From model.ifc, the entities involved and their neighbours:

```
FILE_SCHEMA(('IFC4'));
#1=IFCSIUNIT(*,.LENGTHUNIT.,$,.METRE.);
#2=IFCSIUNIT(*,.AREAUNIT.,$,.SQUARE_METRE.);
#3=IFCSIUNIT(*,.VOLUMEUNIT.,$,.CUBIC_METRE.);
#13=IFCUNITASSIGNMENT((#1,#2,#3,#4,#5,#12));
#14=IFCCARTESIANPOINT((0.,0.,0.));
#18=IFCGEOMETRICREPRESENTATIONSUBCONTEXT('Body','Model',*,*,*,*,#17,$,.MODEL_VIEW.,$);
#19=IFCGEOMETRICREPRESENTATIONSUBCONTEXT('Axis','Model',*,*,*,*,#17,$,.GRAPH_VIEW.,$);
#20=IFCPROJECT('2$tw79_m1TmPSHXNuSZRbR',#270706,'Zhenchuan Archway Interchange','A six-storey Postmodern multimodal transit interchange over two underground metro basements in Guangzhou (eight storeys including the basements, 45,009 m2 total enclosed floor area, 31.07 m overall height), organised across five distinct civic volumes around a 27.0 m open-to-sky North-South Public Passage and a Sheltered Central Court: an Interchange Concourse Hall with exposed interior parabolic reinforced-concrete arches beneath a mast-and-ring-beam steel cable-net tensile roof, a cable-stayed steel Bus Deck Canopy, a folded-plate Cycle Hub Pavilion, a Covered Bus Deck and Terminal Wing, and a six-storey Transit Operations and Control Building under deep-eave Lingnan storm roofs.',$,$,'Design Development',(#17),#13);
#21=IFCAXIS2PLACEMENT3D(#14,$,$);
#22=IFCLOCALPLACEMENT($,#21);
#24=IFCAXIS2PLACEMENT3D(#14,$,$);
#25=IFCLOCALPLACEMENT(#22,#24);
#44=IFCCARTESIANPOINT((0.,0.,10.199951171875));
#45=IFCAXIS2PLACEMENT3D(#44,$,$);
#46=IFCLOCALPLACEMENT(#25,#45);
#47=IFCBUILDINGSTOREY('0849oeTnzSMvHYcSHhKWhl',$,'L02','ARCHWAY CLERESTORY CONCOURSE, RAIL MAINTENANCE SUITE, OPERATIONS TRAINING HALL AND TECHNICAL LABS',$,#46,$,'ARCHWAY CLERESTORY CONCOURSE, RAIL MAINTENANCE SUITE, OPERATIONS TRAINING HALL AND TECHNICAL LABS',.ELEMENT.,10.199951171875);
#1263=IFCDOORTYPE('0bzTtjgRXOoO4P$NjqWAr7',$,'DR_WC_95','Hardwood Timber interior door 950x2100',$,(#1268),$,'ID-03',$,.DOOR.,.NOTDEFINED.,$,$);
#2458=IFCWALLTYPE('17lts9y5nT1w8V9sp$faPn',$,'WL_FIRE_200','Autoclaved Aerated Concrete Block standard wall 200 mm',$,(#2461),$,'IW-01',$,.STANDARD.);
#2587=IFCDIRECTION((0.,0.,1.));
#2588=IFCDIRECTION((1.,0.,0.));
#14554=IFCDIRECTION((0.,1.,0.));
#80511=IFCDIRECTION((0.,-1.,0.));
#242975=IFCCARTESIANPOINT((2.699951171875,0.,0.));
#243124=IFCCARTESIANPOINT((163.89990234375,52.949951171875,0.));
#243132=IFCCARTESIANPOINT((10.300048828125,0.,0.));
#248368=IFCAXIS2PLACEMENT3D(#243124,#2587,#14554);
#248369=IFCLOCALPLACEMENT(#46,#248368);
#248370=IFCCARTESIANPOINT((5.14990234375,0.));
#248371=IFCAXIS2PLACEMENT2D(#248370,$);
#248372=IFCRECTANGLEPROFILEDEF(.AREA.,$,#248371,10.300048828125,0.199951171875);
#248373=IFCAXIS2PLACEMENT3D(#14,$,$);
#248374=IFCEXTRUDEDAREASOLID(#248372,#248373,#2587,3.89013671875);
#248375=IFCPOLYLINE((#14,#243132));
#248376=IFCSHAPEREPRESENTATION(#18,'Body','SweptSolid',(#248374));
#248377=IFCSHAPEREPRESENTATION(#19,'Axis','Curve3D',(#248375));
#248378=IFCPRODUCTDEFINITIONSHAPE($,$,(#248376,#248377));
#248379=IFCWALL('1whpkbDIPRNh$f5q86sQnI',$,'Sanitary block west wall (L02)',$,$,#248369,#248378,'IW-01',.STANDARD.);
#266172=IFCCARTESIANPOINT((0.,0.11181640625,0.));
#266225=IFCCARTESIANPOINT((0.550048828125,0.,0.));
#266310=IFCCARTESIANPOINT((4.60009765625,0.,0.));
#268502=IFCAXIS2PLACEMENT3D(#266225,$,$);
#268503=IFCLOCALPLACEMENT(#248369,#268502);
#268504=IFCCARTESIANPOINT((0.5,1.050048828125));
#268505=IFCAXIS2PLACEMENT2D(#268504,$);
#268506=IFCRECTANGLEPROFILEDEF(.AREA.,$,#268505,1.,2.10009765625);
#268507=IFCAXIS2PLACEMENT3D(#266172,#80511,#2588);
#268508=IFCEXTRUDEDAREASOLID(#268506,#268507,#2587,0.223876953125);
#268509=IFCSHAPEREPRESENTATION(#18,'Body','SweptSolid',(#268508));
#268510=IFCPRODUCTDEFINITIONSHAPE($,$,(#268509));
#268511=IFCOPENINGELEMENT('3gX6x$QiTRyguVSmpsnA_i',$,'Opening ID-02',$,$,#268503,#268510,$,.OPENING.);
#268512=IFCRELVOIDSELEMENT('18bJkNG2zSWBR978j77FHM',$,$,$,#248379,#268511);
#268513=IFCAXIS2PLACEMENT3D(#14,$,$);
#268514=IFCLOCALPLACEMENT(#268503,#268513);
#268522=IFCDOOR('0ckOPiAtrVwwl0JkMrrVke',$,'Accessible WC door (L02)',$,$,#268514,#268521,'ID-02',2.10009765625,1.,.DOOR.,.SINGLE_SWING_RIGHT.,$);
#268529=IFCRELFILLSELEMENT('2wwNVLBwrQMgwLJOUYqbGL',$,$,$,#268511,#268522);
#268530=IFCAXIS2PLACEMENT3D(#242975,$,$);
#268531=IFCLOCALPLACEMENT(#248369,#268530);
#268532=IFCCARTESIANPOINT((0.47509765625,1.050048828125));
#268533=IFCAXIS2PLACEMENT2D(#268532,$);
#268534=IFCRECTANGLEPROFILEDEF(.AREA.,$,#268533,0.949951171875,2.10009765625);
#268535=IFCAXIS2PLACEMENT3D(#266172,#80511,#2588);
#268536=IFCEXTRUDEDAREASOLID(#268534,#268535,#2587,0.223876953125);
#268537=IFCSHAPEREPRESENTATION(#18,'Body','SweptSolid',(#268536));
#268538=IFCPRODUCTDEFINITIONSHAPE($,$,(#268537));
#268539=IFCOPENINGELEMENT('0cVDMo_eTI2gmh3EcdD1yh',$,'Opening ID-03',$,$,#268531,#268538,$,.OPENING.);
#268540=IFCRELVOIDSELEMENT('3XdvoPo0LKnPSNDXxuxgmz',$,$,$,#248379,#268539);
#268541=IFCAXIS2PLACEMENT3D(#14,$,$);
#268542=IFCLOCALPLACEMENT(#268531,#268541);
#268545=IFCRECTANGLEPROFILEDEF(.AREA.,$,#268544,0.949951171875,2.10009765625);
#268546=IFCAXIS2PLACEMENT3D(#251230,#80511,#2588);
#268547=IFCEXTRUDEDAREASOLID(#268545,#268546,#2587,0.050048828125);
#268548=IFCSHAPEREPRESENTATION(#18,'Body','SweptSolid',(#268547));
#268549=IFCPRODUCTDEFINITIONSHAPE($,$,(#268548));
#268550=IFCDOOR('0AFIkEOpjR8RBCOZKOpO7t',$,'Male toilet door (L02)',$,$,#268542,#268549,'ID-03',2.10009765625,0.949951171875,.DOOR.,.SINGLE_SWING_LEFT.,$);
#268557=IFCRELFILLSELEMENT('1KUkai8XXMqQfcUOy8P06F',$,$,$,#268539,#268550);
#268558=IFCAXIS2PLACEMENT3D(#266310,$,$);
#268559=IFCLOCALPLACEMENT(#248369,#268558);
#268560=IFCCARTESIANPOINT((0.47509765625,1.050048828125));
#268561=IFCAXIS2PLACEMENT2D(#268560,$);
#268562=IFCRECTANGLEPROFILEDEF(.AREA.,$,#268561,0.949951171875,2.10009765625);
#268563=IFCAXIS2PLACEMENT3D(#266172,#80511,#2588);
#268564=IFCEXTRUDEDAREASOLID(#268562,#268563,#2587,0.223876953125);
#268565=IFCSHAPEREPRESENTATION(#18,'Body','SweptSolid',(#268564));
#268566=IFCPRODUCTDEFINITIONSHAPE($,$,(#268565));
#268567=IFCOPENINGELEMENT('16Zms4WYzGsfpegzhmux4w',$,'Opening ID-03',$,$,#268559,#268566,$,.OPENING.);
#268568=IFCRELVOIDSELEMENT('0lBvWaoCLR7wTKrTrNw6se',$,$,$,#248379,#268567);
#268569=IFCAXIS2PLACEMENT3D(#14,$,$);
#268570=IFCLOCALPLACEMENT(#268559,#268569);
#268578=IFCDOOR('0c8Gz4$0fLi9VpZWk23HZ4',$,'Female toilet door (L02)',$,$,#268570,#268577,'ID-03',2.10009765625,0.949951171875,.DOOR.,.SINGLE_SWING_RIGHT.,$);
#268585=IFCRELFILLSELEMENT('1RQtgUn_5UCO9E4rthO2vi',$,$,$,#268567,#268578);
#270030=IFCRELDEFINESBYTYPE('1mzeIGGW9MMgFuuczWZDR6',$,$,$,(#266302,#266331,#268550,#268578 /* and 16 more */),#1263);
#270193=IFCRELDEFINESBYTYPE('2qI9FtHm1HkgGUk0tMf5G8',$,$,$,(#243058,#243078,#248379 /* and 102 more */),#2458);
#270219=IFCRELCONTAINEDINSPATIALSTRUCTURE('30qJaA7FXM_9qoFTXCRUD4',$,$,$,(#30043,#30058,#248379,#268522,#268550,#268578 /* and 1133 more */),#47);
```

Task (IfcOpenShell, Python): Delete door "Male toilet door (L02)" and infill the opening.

```python
import ifcopenshell
import ifcopenshell.api.feature
import ifcopenshell.api.root
import ifcopenshell.geom
import ifcopenshell.util.shape

model = ifcopenshell.open("model.ifc")
settings = ifcopenshell.geom.settings()


def volume(element):
    """Net volume in cubic metres, openings subtracted."""
    shape = ifcopenshell.geom.create_shape(settings, element)
    return ifcopenshell.util.shape.get_volume(shape.geometry)


door = model.by_id(268550)
opening = door.FillsVoids[0].RelatingOpeningElement
wall = opening.VoidsElements[0].RelatingBuildingElement
before = volume(wall)

ifcopenshell.api.root.remove_product(model, product=door)
ifcopenshell.api.feature.remove_feature(model, feature=opening)

after = volume(wall)

print(f"wall volume {before:.3f} -> {after:.3f} m3")

model.write("model_updated.ifc")
```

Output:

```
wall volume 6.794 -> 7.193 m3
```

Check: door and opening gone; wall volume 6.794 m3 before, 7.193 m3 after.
